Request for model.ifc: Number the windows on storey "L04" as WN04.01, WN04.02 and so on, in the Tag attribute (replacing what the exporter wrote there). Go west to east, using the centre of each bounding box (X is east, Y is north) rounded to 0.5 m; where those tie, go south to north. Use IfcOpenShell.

First a look at what the model holds.

```python
import ifcopenshell
import ifcopenshell.util.element
import ifcopenshell.util.placement

model = ifcopenshell.open("model.ifc")
print(model.schema)
storey = next(s for s in model.by_type("IfcBuildingStorey") if s.Name == "L04")
windows = [e for e in ifcopenshell.util.element.get_decomposition(storey) if e.is_a("IfcWindow")]
for e in sorted(windows, key=lambda e: e.id()):
    origin = ifcopenshell.util.placement.get_local_placement(e.ObjectPlacement)[:3, 3]
    print(e.id(), e.Tag, e.Name, origin.round(2) + 0.0, sep=" | ")
```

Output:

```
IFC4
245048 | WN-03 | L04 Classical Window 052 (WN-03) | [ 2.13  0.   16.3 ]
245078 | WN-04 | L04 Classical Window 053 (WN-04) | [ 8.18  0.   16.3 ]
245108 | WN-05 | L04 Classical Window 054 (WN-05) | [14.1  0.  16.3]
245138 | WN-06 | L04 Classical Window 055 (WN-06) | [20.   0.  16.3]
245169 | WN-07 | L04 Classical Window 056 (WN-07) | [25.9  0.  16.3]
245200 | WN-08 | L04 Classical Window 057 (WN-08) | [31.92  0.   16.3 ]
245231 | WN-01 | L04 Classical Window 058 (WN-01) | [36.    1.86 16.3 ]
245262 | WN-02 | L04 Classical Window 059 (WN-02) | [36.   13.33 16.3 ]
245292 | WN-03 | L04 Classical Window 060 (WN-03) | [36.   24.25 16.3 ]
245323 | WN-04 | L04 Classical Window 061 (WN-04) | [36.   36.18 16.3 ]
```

```python
import ifcopenshell
import ifcopenshell.geom
import ifcopenshell.util.element
import ifcopenshell.util.shape

model = ifcopenshell.open("model.ifc")
settings = ifcopenshell.geom.settings()
settings.set("use-world-coords", True)


def centre(element):
    shape = ifcopenshell.geom.create_shape(settings, element)
    return ifcopenshell.util.shape.get_bbox_centroid(shape.geometry)


storey = next(s for s in model.by_type("IfcBuildingStorey") if s.Name == "L04")
windows = [e for e in ifcopenshell.util.element.get_decomposition(storey) if e.is_a("IfcWindow")]

# Insertion points can sit at a corner or the storey origin, so sort by the geometry (in metres).
centres = {e: centre(e) for e in windows}
windows.sort(key=lambda e: (round(centres[e][0] / 0.5), centres[e][1]))

for i, e in enumerate(windows, start=1):
    number = f"WN04.{i:02d}"
    e.Tag = number
    print(e.id(), number)

model.write("model-out.ifc")
```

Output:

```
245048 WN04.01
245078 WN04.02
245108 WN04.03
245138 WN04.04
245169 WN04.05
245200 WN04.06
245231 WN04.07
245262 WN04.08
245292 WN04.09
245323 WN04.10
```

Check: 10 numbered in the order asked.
